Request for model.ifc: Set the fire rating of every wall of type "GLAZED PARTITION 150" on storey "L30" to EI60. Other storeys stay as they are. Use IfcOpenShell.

First a look at what the model holds.

```python
import ifcopenshell
import ifcopenshell.util.element

model = ifcopenshell.open("model.ifc")
print(model.schema)
storey = next(s for s in model.by_type("IfcBuildingStorey") if s.Name == "L30")
walls = [e for e in ifcopenshell.util.element.get_decomposition(storey) if e.is_a("IfcWall")]
seen = {}
for e in walls:
    element_type = ifcopenshell.util.element.get_type(e)
    key = (element_type.Name if element_type != e and element_type else None, ifcopenshell.util.element.get_pset(e, "Pset_WallCommon", "FireRating"))
    seen[key] = seen.get(key, 0) + 1
for (name, value), count in sorted(seen.items(), key=str):
    print(count, "x", name, "|", value)
```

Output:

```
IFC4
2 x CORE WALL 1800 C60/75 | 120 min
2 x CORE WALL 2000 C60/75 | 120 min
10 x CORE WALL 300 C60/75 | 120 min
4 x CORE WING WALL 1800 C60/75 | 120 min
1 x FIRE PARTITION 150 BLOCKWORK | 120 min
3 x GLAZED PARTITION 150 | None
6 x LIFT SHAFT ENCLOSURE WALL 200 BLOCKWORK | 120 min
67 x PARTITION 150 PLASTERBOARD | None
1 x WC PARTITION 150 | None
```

```python
import ifcopenshell
import ifcopenshell.api.pset
import ifcopenshell.util.element

model = ifcopenshell.open("model.ifc")

storey = next(s for s in model.by_type("IfcBuildingStorey") if s.Name == "L30")
walls = [e for e in ifcopenshell.util.element.get_decomposition(storey) if e.is_a("IfcWall")]

count = 0
for e in walls:
    element_type = ifcopenshell.util.element.get_type(e)
    if element_type in (None, e) or element_type.Name != "GLAZED PARTITION 150":
        continue
    # add_pset returns the element's existing set when there is one.
    pset = ifcopenshell.api.pset.add_pset(model, product=e, name="Pset_WallCommon")
    ifcopenshell.api.pset.edit_pset(model, pset=pset, properties={"FireRating": "EI60"})
    count += 1

print(count, "walls updated")

model.write("model_rev.ifc")
```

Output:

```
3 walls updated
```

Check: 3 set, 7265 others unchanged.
